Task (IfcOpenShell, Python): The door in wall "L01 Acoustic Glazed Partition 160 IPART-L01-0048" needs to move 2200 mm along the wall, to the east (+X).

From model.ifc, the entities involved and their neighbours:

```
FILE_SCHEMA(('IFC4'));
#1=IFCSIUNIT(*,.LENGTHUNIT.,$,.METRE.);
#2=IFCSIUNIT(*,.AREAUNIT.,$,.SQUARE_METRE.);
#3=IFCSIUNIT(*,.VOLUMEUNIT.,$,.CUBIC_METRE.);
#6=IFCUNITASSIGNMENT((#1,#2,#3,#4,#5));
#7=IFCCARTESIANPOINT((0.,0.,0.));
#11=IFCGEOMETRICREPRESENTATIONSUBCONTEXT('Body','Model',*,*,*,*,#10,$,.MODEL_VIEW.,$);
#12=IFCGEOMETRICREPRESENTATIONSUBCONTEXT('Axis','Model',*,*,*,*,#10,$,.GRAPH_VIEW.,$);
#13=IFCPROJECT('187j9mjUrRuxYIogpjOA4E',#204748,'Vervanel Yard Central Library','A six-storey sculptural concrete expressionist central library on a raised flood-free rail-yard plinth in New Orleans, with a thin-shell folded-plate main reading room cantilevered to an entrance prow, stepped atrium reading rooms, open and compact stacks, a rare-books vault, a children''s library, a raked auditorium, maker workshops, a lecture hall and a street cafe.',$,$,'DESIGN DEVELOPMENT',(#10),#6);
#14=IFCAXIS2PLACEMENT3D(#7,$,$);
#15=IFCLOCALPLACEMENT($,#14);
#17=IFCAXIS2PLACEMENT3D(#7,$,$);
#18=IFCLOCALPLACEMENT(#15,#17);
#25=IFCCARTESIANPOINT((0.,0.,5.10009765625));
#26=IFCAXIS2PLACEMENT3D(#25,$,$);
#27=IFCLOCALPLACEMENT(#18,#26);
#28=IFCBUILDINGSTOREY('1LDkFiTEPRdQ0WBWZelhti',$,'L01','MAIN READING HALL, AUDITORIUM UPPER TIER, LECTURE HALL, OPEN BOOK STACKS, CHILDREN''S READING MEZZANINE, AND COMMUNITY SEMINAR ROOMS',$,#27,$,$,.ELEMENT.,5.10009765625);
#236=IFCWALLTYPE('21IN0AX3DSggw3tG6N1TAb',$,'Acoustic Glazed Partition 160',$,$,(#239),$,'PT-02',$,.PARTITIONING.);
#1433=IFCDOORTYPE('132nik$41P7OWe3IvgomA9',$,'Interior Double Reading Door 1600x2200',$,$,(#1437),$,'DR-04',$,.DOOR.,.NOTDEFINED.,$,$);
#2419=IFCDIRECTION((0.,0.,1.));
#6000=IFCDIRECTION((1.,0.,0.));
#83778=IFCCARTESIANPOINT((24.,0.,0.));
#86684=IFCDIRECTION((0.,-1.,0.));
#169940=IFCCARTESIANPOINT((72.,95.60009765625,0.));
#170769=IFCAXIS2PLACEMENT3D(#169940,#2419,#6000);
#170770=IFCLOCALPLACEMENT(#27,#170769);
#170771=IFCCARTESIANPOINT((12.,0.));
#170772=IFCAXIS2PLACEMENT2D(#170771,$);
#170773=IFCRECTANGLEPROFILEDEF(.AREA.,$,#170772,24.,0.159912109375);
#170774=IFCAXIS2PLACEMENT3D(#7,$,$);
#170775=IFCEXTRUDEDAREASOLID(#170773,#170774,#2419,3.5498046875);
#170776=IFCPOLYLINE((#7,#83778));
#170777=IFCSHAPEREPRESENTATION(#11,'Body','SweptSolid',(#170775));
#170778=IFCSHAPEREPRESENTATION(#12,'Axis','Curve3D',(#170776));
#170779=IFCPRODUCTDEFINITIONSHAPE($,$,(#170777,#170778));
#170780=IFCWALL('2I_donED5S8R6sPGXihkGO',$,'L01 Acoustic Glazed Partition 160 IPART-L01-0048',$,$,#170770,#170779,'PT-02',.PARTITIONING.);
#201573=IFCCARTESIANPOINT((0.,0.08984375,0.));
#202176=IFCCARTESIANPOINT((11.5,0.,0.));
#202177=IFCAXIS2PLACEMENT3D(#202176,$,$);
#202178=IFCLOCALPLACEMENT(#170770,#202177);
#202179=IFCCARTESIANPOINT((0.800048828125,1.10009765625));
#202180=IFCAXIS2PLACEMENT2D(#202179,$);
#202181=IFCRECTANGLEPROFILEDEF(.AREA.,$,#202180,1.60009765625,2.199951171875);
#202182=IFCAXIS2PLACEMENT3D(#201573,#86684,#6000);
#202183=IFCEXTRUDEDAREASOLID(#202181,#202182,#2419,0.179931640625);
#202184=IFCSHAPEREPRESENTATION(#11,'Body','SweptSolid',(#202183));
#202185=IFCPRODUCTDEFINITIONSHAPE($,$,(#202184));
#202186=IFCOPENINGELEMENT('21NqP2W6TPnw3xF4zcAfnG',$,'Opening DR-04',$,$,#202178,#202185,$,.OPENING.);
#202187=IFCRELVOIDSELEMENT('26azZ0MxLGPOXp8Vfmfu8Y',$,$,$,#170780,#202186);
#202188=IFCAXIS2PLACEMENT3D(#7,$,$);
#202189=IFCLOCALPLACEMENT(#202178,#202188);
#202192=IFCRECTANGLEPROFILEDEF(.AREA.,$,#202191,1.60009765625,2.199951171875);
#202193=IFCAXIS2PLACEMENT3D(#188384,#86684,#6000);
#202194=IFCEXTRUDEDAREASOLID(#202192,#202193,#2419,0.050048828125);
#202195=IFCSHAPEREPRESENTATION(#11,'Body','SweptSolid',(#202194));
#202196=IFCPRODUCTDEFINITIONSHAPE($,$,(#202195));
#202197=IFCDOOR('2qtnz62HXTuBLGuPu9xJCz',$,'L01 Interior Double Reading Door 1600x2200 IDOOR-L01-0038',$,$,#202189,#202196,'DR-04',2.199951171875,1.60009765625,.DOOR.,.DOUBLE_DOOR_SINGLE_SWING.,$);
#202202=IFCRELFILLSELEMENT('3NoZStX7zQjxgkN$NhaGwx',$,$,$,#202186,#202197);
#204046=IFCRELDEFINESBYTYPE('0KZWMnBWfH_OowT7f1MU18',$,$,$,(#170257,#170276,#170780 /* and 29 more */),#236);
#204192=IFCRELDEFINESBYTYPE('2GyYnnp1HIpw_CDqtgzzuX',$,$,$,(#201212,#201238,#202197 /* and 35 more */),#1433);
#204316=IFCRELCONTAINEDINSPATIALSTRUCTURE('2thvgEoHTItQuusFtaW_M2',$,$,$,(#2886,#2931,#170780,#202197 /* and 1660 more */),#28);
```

```python
import ifcopenshell
import ifcopenshell.api.geometry
import ifcopenshell.util.placement

model = ifcopenshell.open("model.ifc")

door = model.by_guid("2qtnz62HXTuBLGuPu9xJCz")
opening = door.FillsVoids[0].RelatingOpeningElement
wall = opening.VoidsElements[0].RelatingBuildingElement

wall_matrix = ifcopenshell.util.placement.get_local_placement(wall.ObjectPlacement)
shift = wall_matrix[:3, 0] * 2.2
before = ifcopenshell.util.placement.get_local_placement(door.ObjectPlacement)[:3, 3].copy()

# The door is placed relative to its opening, so it follows when the opening moves.
matrix = ifcopenshell.util.placement.get_local_placement(opening.ObjectPlacement)
matrix[:3, 3] += shift
ifcopenshell.api.geometry.edit_object_placement(
    model, product=opening, matrix=matrix, is_si=False, should_transform_children=True
)

after = ifcopenshell.util.placement.get_local_placement(door.ObjectPlacement)[:3, 3]
print("door moved by", (after - before).round(3) + 0.0)

model.write("model-out.ifc")
```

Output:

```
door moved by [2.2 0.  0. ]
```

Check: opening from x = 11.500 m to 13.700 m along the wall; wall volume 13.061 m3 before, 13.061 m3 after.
